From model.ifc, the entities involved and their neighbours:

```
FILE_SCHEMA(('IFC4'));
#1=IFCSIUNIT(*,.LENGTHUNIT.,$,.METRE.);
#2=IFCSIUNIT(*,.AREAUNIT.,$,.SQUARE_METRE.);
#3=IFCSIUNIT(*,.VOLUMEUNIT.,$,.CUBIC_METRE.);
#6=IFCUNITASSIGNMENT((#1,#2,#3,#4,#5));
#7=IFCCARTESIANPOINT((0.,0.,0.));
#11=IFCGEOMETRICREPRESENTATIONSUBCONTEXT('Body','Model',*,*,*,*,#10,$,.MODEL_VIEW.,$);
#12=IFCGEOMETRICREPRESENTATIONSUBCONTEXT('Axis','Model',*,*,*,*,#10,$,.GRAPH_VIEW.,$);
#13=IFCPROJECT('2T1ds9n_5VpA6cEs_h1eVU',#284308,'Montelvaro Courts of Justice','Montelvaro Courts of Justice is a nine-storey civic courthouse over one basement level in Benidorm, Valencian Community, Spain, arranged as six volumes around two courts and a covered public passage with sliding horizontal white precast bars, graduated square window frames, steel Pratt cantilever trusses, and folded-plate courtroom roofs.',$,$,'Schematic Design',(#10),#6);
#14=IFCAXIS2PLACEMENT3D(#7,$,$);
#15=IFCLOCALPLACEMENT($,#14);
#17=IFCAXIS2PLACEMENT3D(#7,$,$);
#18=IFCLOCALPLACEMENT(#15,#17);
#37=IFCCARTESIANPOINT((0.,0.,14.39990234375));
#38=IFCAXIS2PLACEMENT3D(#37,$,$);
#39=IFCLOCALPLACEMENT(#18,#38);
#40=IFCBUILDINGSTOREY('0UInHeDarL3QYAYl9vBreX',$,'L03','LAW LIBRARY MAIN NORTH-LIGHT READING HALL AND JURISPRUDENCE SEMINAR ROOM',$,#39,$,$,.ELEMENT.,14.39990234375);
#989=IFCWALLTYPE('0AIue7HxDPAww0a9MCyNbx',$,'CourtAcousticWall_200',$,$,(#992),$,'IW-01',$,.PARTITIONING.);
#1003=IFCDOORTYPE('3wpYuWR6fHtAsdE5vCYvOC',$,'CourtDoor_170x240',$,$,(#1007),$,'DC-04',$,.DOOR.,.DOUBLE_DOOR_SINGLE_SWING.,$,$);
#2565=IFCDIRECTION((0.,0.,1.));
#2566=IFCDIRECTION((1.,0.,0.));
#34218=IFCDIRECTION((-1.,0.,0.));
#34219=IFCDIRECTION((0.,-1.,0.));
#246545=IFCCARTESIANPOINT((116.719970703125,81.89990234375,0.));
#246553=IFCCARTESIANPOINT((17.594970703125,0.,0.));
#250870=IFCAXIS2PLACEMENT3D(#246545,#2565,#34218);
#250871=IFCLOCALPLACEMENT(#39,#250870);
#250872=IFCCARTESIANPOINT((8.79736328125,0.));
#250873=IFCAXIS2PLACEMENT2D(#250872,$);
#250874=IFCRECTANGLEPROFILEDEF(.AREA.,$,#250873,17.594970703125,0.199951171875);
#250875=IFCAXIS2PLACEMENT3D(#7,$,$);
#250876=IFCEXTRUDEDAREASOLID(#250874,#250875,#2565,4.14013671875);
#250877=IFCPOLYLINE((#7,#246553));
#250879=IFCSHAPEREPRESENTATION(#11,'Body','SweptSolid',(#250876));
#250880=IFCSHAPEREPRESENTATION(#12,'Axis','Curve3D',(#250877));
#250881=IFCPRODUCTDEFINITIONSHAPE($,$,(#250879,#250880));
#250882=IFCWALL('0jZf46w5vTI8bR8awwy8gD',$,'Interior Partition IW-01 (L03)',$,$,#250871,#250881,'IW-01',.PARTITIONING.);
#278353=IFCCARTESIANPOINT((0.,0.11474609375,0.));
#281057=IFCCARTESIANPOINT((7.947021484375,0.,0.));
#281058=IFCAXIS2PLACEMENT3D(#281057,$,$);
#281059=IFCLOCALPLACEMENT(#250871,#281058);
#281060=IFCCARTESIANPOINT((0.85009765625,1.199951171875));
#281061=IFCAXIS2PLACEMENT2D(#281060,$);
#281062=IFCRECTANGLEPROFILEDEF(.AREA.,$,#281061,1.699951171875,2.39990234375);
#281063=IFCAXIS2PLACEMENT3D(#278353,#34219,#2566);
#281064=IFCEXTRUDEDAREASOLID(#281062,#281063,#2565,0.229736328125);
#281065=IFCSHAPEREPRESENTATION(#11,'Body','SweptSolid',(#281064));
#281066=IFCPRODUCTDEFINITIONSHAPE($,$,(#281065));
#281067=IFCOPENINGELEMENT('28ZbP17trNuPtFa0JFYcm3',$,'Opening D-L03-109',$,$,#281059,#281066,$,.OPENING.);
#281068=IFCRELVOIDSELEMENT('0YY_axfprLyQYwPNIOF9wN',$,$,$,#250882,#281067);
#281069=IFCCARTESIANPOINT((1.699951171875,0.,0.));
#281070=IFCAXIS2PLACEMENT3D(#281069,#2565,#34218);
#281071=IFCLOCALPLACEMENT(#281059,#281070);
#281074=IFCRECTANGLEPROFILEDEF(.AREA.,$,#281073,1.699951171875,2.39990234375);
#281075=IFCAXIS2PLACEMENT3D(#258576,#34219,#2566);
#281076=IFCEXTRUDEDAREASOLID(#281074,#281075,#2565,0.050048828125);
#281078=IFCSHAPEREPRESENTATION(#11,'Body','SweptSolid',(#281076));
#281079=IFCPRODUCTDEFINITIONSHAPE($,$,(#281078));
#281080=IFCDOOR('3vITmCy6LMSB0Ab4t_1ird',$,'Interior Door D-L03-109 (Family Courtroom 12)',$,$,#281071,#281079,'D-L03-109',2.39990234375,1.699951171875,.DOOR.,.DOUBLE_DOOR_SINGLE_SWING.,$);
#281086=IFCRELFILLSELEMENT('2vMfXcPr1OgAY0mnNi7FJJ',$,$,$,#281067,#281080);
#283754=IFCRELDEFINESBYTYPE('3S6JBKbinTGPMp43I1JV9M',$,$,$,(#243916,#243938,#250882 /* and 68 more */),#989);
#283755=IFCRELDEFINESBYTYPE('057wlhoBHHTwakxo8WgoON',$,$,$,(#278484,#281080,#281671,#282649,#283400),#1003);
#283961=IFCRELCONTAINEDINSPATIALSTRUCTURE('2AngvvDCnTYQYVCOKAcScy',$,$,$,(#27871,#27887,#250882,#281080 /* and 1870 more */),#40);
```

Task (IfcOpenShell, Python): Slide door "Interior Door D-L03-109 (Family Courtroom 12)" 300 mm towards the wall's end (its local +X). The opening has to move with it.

```python
import ifcopenshell
import ifcopenshell.api.geometry
import ifcopenshell.util.placement

model = ifcopenshell.open("model.ifc")

door = model.by_guid("3vITmCy6LMSB0Ab4t_1ird")
opening = door.FillsVoids[0].RelatingOpeningElement
wall = opening.VoidsElements[0].RelatingBuildingElement

wall_matrix = ifcopenshell.util.placement.get_local_placement(wall.ObjectPlacement)
shift = wall_matrix[:3, 0] * 0.3
before = ifcopenshell.util.placement.get_local_placement(door.ObjectPlacement)[:3, 3].copy()

# The door is placed relative to its opening, so it follows when the opening moves.
matrix = ifcopenshell.util.placement.get_local_placement(opening.ObjectPlacement)
matrix[:3, 3] += shift
ifcopenshell.api.geometry.edit_object_placement(
    model, product=opening, matrix=matrix, is_si=False, should_transform_children=True
)

after = ifcopenshell.util.placement.get_local_placement(door.ObjectPlacement)[:3, 3]
print("door moved by", (after - before).round(3) + 0.0)

model.write("model_v2.ifc")
```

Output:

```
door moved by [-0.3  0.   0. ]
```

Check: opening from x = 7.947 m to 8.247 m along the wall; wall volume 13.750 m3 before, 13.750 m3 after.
